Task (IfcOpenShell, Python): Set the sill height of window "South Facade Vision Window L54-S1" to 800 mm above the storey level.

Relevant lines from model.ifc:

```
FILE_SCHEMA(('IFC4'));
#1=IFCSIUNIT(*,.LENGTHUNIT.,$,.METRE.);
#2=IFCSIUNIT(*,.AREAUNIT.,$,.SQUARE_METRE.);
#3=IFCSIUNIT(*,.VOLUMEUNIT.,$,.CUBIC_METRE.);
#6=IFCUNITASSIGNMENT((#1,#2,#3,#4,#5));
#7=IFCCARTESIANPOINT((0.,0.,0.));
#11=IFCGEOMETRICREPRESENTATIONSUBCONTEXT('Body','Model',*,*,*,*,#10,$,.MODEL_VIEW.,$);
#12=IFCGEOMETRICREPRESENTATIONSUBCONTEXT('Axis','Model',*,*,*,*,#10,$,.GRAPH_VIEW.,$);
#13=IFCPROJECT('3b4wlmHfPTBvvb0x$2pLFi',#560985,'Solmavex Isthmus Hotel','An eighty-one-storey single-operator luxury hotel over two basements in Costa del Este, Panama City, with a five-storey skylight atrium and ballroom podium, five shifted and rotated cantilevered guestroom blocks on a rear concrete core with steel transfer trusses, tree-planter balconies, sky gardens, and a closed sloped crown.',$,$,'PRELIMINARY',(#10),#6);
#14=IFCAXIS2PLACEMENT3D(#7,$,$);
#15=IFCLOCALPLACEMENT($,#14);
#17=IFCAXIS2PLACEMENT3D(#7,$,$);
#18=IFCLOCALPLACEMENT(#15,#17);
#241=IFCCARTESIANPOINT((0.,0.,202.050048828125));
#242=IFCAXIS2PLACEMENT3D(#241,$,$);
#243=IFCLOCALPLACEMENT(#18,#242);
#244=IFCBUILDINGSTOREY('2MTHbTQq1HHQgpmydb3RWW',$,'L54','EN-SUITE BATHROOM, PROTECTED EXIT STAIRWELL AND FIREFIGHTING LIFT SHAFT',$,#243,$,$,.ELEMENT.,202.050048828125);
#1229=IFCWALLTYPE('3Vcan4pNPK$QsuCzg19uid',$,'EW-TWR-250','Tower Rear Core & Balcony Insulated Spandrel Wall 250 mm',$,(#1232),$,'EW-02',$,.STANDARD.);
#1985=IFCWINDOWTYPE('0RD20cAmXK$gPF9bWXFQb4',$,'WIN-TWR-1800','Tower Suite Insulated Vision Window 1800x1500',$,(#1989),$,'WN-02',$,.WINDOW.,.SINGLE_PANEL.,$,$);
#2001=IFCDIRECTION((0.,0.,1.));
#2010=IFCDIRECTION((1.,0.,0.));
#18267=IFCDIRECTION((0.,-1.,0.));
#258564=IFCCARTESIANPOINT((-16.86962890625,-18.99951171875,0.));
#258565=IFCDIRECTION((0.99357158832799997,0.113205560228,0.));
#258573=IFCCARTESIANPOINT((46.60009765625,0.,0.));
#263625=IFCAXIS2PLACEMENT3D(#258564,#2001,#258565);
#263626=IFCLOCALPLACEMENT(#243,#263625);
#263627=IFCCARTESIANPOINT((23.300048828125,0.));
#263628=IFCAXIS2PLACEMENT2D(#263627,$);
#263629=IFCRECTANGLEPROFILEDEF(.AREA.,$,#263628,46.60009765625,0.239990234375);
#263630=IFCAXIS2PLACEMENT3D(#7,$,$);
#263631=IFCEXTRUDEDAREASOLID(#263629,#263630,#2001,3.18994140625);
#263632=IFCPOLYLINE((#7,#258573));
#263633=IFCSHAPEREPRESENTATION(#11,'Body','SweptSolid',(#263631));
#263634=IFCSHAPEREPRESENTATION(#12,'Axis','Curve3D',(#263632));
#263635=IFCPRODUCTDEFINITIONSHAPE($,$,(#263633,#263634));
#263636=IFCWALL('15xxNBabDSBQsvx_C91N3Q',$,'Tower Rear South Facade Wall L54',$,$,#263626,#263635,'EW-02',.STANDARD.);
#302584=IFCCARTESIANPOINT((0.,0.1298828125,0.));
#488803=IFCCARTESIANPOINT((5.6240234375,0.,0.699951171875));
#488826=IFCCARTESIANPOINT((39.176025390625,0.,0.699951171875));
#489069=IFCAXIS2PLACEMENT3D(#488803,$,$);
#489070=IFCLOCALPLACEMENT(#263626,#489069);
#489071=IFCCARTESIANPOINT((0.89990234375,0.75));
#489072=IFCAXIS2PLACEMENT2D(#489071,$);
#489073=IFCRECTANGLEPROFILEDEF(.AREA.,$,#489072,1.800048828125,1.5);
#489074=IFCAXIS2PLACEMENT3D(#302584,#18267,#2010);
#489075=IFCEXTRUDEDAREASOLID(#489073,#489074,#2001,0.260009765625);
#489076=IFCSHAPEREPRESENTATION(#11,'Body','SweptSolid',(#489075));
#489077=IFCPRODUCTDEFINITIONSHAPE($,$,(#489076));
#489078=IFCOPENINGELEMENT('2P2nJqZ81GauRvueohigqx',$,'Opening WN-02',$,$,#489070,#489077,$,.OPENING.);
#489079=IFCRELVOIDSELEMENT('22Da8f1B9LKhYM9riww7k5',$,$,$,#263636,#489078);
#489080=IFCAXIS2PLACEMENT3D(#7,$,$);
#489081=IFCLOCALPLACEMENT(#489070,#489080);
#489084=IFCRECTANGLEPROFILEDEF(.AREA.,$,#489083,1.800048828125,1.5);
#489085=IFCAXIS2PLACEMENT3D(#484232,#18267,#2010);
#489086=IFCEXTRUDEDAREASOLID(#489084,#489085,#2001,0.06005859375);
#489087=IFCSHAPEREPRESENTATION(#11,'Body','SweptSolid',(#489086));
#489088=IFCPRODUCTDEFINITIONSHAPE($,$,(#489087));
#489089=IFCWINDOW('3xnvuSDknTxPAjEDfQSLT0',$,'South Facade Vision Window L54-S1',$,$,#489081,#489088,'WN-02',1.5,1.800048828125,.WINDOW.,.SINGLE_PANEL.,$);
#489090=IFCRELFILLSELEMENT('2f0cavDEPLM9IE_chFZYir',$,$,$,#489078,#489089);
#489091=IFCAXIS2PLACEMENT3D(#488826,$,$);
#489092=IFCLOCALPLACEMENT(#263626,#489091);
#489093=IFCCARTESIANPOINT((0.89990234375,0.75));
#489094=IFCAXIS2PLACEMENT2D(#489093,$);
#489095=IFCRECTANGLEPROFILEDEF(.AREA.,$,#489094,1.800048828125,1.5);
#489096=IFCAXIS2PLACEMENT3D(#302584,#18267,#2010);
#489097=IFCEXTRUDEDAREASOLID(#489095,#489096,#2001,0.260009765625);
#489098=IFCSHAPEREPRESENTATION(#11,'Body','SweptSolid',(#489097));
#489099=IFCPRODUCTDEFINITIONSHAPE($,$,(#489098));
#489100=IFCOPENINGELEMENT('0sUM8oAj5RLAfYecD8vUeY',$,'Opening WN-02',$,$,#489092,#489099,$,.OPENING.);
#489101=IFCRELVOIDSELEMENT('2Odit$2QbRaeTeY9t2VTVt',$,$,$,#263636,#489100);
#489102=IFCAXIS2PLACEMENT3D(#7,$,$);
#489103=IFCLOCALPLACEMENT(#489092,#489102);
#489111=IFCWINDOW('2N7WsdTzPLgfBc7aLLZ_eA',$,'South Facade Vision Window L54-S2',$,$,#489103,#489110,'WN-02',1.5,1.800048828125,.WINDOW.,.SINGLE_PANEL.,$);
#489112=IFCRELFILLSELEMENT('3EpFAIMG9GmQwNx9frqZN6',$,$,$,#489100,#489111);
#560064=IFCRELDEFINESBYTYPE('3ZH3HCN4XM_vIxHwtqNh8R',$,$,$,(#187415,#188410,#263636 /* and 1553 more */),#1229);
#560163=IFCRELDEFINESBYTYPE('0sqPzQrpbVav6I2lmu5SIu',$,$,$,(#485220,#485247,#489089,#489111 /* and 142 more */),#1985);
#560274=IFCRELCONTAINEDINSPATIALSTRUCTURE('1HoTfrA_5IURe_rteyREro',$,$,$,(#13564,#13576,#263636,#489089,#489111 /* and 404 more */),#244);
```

```python
import numpy as np
import ifcopenshell
import ifcopenshell.api.geometry
import ifcopenshell.geom
import ifcopenshell.util.element
import ifcopenshell.util.placement
import ifcopenshell.util.shape
import ifcopenshell.util.unit

model = ifcopenshell.open("model.ifc")
unit_scale = ifcopenshell.util.unit.calculate_unit_scale(model)

window = model.by_guid("3xnvuSDknTxPAjEDfQSLT0")
opening = window.FillsVoids[0].RelatingOpeningElement
storey = ifcopenshell.util.element.get_container(window, ifc_class="IfcBuildingStorey")
level = ifcopenshell.util.placement.get_local_placement(storey.ObjectPlacement)[2, 3]

# The opening's origin need not be at the sill, so measure its lowest point.
shape = ifcopenshell.geom.create_shape(ifcopenshell.geom.settings(), opening)
bottom = ifcopenshell.util.shape.get_shape_bottom_elevation(shape, shape.geometry) / unit_scale
dz = level + 0.8 / unit_scale - bottom

shift = np.array([0.0, 0.0, dz])
# The window is placed relative to its opening, so it follows when the opening moves.
matrix = ifcopenshell.util.placement.get_local_placement(opening.ObjectPlacement)
matrix[:3, 3] += shift
ifcopenshell.api.geometry.edit_object_placement(
    model, product=opening, matrix=matrix, is_si=False, should_transform_children=True
)

print(f"moved by {dz * unit_scale:+.3f} m")

model.write("model_edited.ifc")
```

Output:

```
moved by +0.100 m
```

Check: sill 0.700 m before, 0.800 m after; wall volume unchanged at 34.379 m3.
